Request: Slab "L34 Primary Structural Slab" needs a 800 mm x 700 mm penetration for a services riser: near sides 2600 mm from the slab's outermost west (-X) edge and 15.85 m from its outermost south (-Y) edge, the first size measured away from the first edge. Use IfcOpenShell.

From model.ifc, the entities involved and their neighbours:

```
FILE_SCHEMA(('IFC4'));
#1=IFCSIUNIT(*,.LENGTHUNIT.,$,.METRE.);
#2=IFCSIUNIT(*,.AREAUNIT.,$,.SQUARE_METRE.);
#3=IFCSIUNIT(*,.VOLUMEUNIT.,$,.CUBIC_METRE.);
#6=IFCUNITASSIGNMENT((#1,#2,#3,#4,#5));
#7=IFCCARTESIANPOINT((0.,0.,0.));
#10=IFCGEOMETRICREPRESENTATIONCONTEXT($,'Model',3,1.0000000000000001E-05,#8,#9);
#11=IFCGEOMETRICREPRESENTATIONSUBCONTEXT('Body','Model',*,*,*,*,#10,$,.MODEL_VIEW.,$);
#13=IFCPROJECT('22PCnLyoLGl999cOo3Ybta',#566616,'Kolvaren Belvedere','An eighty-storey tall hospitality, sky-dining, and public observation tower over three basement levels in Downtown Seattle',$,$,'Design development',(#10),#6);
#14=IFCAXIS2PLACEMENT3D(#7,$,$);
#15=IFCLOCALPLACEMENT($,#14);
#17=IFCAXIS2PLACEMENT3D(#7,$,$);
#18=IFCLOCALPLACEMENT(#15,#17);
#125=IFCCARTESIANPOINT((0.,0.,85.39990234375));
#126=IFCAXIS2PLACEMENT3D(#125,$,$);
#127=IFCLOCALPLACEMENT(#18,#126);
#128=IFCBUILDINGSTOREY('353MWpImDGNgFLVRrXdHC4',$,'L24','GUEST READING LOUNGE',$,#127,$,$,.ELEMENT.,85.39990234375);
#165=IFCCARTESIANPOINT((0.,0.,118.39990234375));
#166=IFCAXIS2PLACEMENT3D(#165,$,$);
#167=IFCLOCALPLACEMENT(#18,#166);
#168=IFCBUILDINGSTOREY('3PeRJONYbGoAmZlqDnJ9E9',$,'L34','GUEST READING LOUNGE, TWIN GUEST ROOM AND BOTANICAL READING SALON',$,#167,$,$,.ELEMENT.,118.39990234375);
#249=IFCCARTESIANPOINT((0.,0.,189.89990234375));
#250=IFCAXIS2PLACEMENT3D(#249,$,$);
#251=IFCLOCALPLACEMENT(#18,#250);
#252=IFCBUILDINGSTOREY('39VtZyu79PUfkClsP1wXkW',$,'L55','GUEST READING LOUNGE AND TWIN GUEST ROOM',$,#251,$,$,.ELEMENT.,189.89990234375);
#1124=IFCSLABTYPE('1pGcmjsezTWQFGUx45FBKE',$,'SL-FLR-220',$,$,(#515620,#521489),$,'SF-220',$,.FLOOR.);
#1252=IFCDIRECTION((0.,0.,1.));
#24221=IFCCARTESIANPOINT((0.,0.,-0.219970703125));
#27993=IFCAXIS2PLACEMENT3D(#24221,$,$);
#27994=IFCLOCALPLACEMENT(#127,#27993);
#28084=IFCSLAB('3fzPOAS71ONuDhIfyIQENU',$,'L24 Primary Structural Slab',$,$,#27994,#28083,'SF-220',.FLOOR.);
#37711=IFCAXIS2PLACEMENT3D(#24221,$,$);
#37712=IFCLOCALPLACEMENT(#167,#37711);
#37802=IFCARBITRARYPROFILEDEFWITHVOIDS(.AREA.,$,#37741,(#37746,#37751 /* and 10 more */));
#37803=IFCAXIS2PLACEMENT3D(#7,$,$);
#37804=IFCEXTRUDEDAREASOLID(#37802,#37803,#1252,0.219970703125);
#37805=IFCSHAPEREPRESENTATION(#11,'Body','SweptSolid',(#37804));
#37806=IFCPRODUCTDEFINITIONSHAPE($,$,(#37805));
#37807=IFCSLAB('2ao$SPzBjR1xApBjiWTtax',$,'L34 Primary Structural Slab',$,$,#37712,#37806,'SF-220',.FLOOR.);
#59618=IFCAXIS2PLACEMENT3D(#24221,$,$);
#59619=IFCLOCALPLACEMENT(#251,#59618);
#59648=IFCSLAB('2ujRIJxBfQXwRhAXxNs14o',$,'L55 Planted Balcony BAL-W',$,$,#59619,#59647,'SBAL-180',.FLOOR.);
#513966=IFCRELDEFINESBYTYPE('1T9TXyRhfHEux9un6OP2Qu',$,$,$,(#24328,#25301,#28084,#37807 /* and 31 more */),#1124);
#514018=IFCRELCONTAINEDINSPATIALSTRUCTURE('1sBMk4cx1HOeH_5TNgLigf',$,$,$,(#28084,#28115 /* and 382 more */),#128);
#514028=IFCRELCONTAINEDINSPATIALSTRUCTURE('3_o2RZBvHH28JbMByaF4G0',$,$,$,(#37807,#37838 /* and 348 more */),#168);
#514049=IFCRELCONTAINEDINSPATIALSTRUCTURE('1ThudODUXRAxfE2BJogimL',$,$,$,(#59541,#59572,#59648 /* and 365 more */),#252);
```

```python
import numpy as np
import ifcopenshell
import ifcopenshell.api.feature
import ifcopenshell.api.geometry
import ifcopenshell.api.root
import ifcopenshell.geom
import ifcopenshell.util.placement
import ifcopenshell.util.representation
import ifcopenshell.util.shape
import ifcopenshell.util.unit

model = ifcopenshell.open("model.ifc")
unit_scale = ifcopenshell.util.unit.calculate_unit_scale(model)
settings = ifcopenshell.geom.settings()


def volume(element):
    """Net volume in cubic metres, openings subtracted."""
    shape = ifcopenshell.geom.create_shape(settings, element)
    return ifcopenshell.util.shape.get_volume(shape.geometry)


slab = model.by_guid("2ao$SPzBjR1xApBjiWTtax")
before = volume(slab)

# Extent in the slab's own axes, in metres. The edges named are its -X and -Y sides.
slab_shape = ifcopenshell.geom.create_shape(settings, slab)
vertices = ifcopenshell.util.shape.get_vertices(slab_shape.geometry)
x_min, y_min, bottom = vertices.min(axis=0)
top = vertices[:, 2].max()

opening = ifcopenshell.api.root.create_entity(model, ifc_class="IfcOpeningElement", name="Services riser opening", predefined_type="OPENING")
context = ifcopenshell.util.representation.get_context(model, "Model", "Body", "MODEL_VIEW")
width, depth = 0.8, 0.7
outline = [(0.0, 0.0), (width, 0.0), (width, depth), (0.0, depth), (0.0, 0.0)]
# Overshoot both faces by 50 mm so the cut is clean.
shape = ifcopenshell.api.geometry.add_slab_representation(
    model, context=context, depth=top - bottom + 0.1, polyline=outline
)
ifcopenshell.api.geometry.assign_representation(model, product=opening, representation=shape)

matrix = ifcopenshell.util.placement.get_local_placement(slab.ObjectPlacement)
matrix[:, 3] = matrix @ np.append(np.array([x_min + 2.6, y_min + 15.85, bottom - 0.05]) / unit_scale, 1.0)
ifcopenshell.api.geometry.edit_object_placement(model, product=opening, matrix=matrix, is_si=False)
ifcopenshell.api.feature.add_feature(model, feature=opening, element=slab)

after = volume(slab)

print(f"slab volume {before:.3f} -> {after:.3f} m3")

model.write("model_v2.ifc")
```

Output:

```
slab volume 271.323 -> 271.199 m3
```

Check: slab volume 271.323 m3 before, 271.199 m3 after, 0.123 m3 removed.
